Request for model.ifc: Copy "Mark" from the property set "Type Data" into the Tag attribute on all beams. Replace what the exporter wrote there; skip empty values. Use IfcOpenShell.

First a look at what the model holds.

```python
import ifcopenshell
import ifcopenshell.util.element

model = ifcopenshell.open("model.ifc")
print(model.schema)
beams = model.by_type("IfcBeam")
print(len(beams), "beams")
for e in beams[:8]:
    source = ifcopenshell.util.element.get_pset(e, "Type Data", "Mark")
    target = e.Tag
    print(e.id(), repr(source), repr(target), sep=" | ")
```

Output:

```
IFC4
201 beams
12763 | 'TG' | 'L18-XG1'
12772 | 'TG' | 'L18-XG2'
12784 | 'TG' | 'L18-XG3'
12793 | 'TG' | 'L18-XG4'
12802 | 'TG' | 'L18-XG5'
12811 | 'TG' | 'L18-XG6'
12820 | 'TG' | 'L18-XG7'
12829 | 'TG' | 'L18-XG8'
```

```python
import ifcopenshell
import ifcopenshell.util.element

model = ifcopenshell.open("model.ifc")

count = 0
for e in model.by_type("IfcBeam"):
    value = ifcopenshell.util.element.get_pset(e, "Type Data", "Mark")
    current = e.Tag
    if not value or not value.strip() or current == value:
        continue
    e.Tag = value
    count += 1

print(count, "beams updated")

model.write("model_v2.ifc")
```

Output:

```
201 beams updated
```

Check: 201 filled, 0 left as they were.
